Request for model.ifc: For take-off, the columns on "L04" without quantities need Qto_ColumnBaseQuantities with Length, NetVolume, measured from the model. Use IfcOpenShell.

First a look at what the model holds.

```python
import ifcopenshell
import ifcopenshell.util.element
import ifcopenshell.util.unit

model = ifcopenshell.open("model.ifc")
print(model.schema)
for unit_type in ("LENGTHUNIT", "AREAUNIT", "VOLUMEUNIT"):
    print(unit_type, ifcopenshell.util.unit.calculate_unit_scale(model, unit_type))
storey = next(s for s in model.by_type("IfcBuildingStorey") if s.Name == "L04")
columns = [e for e in ifcopenshell.util.element.get_decomposition(storey) if e.is_a("IfcColumn")]
for e in sorted(columns, key=lambda e: e.id()):
    print(e.id(), e.is_a(), e.Name, list(ifcopenshell.util.element.get_psets(e, qtos_only=True)), sep=" | ")
```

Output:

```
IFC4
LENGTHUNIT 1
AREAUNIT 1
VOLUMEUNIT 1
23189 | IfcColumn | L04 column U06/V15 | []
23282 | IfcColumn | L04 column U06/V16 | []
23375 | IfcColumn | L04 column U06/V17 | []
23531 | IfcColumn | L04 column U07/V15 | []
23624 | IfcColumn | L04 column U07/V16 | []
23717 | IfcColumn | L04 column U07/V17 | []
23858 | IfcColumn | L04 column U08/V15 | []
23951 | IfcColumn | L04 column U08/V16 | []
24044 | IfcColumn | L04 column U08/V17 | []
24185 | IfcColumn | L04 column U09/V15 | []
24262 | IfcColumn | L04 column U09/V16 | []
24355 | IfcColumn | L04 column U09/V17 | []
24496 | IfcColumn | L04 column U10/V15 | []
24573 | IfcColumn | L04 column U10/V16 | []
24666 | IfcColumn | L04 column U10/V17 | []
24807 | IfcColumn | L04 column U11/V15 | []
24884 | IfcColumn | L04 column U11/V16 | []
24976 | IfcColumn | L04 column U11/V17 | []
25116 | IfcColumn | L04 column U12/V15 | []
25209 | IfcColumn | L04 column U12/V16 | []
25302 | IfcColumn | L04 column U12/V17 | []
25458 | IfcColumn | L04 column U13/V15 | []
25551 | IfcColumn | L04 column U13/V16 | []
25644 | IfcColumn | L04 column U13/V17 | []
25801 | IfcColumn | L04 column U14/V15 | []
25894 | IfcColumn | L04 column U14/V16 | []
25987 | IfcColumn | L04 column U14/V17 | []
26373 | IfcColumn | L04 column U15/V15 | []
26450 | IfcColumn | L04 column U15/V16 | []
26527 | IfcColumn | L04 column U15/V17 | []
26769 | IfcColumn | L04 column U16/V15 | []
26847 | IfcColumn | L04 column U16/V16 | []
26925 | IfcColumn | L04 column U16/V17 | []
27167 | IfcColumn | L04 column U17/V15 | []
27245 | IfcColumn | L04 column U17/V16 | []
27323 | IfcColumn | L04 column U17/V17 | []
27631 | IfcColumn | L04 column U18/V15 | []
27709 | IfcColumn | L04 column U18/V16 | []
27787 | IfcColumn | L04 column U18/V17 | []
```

```python
import ifcopenshell
import ifcopenshell.api.pset
import ifcopenshell.geom
import ifcopenshell.util.element
import ifcopenshell.util.shape
import ifcopenshell.util.unit

model = ifcopenshell.open("model.ifc")
unit_scale = ifcopenshell.util.unit.calculate_unit_scale(model)
volume_scale = ifcopenshell.util.unit.calculate_unit_scale(model, "VOLUMEUNIT")
settings = ifcopenshell.geom.settings()

storey = next(s for s in model.by_type("IfcBuildingStorey") if s.Name == "L04")
columns = [e for e in ifcopenshell.util.element.get_decomposition(storey) if e.is_a("IfcColumn")]

for e in sorted(columns, key=lambda e: e.id()):
    if ifcopenshell.util.element.get_psets(e, qtos_only=True, should_inherit=False):
        continue
    # Geometry comes back in metres, in the element's own axes.
    shape = ifcopenshell.geom.create_shape(settings, e)
    values = {
        "Length": ifcopenshell.util.shape.get_z(shape.geometry) / unit_scale,
        "NetVolume": ifcopenshell.util.shape.get_volume(shape.geometry) / volume_scale,
    }
    qto = ifcopenshell.api.pset.add_qto(model, product=e, name="Qto_ColumnBaseQuantities")
    ifcopenshell.api.pset.edit_qto(model, qto=qto, properties=values)
    print(e.id(), {k: round(v, 3) for k, v in values.items()})

model.write("model_rev.ifc")
```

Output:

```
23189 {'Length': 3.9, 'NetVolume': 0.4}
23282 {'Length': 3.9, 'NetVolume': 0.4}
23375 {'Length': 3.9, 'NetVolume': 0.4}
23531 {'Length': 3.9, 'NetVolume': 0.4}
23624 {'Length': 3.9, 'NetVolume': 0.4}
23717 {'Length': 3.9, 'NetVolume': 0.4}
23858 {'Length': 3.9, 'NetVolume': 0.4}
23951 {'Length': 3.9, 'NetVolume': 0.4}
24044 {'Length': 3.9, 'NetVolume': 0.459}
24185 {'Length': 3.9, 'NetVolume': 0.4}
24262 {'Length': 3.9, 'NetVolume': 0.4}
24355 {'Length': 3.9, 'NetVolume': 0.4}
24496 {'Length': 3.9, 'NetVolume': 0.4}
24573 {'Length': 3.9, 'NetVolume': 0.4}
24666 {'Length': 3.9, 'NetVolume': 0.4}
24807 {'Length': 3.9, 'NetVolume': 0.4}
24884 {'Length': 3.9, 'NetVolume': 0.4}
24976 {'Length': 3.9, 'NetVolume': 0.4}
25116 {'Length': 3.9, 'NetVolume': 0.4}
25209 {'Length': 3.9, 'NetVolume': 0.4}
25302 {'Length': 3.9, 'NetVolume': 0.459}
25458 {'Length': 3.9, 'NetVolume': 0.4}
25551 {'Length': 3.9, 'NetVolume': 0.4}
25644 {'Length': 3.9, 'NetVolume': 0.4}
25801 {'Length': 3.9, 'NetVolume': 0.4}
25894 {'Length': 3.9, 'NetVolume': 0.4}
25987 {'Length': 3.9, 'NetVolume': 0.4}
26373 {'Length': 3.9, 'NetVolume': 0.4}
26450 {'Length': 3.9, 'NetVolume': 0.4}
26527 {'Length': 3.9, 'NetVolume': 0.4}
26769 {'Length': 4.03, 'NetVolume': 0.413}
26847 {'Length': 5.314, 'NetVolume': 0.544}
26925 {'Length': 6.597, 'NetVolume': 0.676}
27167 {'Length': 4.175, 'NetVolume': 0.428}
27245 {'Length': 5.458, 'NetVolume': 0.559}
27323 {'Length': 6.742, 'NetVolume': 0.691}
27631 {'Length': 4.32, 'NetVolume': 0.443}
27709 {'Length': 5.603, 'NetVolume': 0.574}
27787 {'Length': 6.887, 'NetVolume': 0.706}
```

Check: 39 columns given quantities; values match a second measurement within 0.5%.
